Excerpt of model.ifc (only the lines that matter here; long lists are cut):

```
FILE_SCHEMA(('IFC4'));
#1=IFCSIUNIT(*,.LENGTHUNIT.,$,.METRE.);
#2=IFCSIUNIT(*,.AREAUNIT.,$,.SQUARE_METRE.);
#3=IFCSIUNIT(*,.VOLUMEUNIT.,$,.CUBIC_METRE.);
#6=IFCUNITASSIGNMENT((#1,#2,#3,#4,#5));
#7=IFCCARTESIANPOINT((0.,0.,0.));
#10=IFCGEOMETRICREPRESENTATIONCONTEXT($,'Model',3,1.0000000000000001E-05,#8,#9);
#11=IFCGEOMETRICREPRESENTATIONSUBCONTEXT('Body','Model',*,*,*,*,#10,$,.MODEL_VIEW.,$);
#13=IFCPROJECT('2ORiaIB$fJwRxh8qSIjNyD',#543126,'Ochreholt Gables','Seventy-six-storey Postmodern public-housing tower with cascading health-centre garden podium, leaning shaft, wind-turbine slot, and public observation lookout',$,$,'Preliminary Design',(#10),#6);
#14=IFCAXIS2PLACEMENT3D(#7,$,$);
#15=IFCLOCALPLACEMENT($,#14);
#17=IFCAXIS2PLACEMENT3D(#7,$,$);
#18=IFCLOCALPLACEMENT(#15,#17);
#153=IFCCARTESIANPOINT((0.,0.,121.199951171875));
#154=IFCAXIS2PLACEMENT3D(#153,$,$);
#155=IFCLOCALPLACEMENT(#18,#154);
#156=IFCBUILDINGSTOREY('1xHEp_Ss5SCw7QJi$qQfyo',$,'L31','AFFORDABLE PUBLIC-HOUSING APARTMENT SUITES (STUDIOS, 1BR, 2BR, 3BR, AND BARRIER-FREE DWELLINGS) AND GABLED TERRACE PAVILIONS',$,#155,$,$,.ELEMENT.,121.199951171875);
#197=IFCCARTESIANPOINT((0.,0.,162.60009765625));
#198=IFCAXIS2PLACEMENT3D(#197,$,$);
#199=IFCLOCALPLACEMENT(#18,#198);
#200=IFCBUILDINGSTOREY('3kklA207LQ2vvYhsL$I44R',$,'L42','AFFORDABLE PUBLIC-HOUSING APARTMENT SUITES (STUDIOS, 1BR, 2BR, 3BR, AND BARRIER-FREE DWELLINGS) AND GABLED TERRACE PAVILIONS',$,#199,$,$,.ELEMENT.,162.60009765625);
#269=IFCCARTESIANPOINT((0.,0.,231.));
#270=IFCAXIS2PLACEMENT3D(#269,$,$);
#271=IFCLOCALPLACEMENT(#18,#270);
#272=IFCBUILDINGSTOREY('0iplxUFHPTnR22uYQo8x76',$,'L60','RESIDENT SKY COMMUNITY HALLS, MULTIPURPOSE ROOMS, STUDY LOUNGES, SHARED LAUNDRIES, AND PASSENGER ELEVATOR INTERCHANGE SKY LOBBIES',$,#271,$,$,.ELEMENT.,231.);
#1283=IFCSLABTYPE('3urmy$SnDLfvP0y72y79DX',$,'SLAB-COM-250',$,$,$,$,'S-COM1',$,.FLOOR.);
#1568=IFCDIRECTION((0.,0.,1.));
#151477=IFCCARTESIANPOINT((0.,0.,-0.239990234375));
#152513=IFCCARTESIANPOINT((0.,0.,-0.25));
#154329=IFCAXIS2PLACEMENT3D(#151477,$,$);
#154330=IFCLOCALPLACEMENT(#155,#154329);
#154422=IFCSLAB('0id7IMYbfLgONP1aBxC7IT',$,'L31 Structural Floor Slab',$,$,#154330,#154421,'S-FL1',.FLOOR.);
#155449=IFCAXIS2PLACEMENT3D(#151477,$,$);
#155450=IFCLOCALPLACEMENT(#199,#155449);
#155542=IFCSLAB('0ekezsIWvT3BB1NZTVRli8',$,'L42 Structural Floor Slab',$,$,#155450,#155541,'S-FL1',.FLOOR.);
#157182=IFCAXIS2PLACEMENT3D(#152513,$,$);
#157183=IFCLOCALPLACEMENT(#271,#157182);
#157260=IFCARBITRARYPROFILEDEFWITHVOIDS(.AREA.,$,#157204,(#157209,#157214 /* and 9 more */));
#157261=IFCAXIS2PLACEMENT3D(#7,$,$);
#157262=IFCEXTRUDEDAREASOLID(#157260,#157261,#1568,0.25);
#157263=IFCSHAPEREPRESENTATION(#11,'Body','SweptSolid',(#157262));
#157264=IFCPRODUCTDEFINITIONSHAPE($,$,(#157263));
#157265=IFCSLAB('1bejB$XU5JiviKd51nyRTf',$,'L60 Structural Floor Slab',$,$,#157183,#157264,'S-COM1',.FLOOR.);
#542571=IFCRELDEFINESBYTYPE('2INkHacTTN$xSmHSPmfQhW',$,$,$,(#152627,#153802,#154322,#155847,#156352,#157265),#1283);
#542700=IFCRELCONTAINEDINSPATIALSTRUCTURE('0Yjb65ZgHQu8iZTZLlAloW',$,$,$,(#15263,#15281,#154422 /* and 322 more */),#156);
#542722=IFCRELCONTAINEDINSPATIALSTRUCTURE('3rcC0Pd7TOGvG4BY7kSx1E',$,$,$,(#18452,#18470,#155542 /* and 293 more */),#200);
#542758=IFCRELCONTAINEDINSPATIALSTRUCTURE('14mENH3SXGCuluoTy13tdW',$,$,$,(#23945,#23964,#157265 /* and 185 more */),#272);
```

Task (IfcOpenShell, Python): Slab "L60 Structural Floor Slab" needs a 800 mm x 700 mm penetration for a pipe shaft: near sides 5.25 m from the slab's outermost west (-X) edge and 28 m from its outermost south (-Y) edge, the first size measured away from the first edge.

```python
import numpy as np
import ifcopenshell
import ifcopenshell.api.feature
import ifcopenshell.api.geometry
import ifcopenshell.api.root
import ifcopenshell.geom
import ifcopenshell.util.placement
import ifcopenshell.util.representation
import ifcopenshell.util.shape
import ifcopenshell.util.unit

model = ifcopenshell.open("model.ifc")
unit_scale = ifcopenshell.util.unit.calculate_unit_scale(model)
settings = ifcopenshell.geom.settings()


def volume(element):
    """Net volume in cubic metres, openings subtracted."""
    shape = ifcopenshell.geom.create_shape(settings, element)
    return ifcopenshell.util.shape.get_volume(shape.geometry)


slab = model.by_id(157265)
before = volume(slab)

# Extent in the slab's own axes, in metres. The edges named are its -X and -Y sides.
slab_shape = ifcopenshell.geom.create_shape(settings, slab)
vertices = ifcopenshell.util.shape.get_vertices(slab_shape.geometry)
x_min, y_min, bottom = vertices.min(axis=0)
top = vertices[:, 2].max()

opening = ifcopenshell.api.root.create_entity(model, ifc_class="IfcOpeningElement", name="Pipe shaft opening", predefined_type="OPENING")
context = ifcopenshell.util.representation.get_context(model, "Model", "Body", "MODEL_VIEW")
width, depth = 0.8, 0.7
outline = [(0.0, 0.0), (width, 0.0), (width, depth), (0.0, depth), (0.0, 0.0)]
# Overshoot both faces by 50 mm so the cut is clean.
shape = ifcopenshell.api.geometry.add_slab_representation(
    model, context=context, depth=top - bottom + 0.1, polyline=outline
)
ifcopenshell.api.geometry.assign_representation(model, product=opening, representation=shape)

matrix = ifcopenshell.util.placement.get_local_placement(slab.ObjectPlacement)
matrix[:, 3] = matrix @ np.append(np.array([x_min + 5.25, y_min + 28, bottom - 0.05]) / unit_scale, 1.0)
ifcopenshell.api.geometry.edit_object_placement(model, product=opening, matrix=matrix, is_si=False)
ifcopenshell.api.feature.add_feature(model, feature=opening, element=slab)

after = volume(slab)

print(f"slab volume {before:.3f} -> {after:.3f} m3")

model.write("model_updated.ifc")
```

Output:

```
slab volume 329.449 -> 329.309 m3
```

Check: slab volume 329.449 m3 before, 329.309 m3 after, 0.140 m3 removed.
